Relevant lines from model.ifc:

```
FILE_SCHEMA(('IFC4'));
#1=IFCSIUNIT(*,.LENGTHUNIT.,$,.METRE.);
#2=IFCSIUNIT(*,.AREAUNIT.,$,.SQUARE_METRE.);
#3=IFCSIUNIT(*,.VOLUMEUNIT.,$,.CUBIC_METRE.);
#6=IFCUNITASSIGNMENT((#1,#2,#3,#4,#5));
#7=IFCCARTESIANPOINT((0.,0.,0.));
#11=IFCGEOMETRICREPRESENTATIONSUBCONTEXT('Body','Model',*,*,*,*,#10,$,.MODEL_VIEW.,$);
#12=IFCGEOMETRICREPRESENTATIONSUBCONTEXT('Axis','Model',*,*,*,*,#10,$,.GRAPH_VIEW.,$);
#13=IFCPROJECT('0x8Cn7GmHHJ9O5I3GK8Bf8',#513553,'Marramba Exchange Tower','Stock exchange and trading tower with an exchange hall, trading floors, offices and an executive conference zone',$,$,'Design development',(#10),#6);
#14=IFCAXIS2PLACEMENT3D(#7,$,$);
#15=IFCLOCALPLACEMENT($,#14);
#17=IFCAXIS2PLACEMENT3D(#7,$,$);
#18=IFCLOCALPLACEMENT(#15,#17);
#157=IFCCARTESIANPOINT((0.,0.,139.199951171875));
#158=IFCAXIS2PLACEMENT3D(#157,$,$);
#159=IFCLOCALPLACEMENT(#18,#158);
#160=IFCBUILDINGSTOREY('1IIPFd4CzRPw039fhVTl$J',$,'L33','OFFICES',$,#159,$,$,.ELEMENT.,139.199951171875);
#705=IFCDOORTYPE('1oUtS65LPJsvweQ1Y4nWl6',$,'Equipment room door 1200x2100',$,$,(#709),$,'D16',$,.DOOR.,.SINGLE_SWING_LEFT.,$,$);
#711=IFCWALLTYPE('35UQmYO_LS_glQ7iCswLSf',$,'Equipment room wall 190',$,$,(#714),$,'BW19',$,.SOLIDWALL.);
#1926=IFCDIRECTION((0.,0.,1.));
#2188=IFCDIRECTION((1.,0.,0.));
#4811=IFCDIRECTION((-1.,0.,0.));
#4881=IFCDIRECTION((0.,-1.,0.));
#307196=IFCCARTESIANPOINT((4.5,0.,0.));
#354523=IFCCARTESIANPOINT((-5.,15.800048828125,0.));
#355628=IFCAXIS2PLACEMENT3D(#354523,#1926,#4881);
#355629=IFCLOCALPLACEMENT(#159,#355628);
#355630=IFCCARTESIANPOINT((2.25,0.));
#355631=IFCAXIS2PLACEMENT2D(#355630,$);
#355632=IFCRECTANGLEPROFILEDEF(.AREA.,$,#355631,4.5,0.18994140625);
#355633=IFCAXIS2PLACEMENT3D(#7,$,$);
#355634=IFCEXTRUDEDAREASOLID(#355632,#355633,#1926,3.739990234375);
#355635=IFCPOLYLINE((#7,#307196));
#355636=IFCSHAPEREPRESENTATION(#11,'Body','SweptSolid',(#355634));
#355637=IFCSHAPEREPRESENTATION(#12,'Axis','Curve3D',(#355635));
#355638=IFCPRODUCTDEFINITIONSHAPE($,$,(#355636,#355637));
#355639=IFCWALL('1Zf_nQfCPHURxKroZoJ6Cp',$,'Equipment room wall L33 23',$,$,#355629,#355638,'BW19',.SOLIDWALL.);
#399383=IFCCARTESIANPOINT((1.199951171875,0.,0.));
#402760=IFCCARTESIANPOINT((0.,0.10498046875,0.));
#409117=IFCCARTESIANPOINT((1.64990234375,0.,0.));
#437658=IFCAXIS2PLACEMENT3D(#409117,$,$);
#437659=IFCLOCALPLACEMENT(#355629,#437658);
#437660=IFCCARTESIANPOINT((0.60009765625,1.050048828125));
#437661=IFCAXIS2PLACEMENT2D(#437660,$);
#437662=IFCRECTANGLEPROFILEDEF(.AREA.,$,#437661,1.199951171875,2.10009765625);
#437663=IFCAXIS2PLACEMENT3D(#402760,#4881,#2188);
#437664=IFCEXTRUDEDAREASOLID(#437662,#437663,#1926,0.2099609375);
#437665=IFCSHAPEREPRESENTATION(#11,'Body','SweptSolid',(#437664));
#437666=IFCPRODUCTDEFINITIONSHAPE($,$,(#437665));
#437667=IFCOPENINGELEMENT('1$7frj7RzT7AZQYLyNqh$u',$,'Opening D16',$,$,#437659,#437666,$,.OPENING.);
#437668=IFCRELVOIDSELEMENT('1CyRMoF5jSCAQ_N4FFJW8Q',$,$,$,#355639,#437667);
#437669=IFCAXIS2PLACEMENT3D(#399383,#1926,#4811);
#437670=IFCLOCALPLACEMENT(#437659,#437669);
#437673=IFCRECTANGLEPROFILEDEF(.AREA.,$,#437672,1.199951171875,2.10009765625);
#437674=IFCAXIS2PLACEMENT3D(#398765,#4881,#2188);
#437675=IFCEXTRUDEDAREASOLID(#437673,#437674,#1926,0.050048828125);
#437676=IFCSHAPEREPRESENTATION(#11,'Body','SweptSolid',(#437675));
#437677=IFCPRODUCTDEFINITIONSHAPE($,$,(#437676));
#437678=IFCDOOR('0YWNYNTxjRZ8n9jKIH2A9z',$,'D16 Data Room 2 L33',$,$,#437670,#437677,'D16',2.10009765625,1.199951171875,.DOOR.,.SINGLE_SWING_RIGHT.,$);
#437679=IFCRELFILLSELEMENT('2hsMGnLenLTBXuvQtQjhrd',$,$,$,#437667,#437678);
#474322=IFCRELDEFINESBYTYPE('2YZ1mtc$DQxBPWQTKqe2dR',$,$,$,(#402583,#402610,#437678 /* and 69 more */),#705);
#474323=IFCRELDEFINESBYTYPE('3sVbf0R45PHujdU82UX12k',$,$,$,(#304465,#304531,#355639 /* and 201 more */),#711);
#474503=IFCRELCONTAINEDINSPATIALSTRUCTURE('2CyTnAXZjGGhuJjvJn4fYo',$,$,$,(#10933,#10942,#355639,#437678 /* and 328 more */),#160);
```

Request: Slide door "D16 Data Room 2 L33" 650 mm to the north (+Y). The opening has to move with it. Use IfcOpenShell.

```python
import ifcopenshell
import ifcopenshell.api.geometry
import ifcopenshell.util.placement

model = ifcopenshell.open("model.ifc")

door = model.by_id(437678)
opening = door.FillsVoids[0].RelatingOpeningElement
wall = opening.VoidsElements[0].RelatingBuildingElement

wall_matrix = ifcopenshell.util.placement.get_local_placement(wall.ObjectPlacement)
shift = wall_matrix[:3, 0] * -0.65
before = ifcopenshell.util.placement.get_local_placement(door.ObjectPlacement)[:3, 3].copy()

# The door is placed relative to its opening, so it follows when the opening moves.
matrix = ifcopenshell.util.placement.get_local_placement(opening.ObjectPlacement)
matrix[:3, 3] += shift
ifcopenshell.api.geometry.edit_object_placement(
    model, product=opening, matrix=matrix, is_si=False, should_transform_children=True
)

after = ifcopenshell.util.placement.get_local_placement(door.ObjectPlacement)[:3, 3]
print("door moved by", (after - before).round(3) + 0.0)

model.write("model-out.ifc")
```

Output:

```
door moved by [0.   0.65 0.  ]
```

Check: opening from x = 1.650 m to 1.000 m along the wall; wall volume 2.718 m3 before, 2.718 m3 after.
